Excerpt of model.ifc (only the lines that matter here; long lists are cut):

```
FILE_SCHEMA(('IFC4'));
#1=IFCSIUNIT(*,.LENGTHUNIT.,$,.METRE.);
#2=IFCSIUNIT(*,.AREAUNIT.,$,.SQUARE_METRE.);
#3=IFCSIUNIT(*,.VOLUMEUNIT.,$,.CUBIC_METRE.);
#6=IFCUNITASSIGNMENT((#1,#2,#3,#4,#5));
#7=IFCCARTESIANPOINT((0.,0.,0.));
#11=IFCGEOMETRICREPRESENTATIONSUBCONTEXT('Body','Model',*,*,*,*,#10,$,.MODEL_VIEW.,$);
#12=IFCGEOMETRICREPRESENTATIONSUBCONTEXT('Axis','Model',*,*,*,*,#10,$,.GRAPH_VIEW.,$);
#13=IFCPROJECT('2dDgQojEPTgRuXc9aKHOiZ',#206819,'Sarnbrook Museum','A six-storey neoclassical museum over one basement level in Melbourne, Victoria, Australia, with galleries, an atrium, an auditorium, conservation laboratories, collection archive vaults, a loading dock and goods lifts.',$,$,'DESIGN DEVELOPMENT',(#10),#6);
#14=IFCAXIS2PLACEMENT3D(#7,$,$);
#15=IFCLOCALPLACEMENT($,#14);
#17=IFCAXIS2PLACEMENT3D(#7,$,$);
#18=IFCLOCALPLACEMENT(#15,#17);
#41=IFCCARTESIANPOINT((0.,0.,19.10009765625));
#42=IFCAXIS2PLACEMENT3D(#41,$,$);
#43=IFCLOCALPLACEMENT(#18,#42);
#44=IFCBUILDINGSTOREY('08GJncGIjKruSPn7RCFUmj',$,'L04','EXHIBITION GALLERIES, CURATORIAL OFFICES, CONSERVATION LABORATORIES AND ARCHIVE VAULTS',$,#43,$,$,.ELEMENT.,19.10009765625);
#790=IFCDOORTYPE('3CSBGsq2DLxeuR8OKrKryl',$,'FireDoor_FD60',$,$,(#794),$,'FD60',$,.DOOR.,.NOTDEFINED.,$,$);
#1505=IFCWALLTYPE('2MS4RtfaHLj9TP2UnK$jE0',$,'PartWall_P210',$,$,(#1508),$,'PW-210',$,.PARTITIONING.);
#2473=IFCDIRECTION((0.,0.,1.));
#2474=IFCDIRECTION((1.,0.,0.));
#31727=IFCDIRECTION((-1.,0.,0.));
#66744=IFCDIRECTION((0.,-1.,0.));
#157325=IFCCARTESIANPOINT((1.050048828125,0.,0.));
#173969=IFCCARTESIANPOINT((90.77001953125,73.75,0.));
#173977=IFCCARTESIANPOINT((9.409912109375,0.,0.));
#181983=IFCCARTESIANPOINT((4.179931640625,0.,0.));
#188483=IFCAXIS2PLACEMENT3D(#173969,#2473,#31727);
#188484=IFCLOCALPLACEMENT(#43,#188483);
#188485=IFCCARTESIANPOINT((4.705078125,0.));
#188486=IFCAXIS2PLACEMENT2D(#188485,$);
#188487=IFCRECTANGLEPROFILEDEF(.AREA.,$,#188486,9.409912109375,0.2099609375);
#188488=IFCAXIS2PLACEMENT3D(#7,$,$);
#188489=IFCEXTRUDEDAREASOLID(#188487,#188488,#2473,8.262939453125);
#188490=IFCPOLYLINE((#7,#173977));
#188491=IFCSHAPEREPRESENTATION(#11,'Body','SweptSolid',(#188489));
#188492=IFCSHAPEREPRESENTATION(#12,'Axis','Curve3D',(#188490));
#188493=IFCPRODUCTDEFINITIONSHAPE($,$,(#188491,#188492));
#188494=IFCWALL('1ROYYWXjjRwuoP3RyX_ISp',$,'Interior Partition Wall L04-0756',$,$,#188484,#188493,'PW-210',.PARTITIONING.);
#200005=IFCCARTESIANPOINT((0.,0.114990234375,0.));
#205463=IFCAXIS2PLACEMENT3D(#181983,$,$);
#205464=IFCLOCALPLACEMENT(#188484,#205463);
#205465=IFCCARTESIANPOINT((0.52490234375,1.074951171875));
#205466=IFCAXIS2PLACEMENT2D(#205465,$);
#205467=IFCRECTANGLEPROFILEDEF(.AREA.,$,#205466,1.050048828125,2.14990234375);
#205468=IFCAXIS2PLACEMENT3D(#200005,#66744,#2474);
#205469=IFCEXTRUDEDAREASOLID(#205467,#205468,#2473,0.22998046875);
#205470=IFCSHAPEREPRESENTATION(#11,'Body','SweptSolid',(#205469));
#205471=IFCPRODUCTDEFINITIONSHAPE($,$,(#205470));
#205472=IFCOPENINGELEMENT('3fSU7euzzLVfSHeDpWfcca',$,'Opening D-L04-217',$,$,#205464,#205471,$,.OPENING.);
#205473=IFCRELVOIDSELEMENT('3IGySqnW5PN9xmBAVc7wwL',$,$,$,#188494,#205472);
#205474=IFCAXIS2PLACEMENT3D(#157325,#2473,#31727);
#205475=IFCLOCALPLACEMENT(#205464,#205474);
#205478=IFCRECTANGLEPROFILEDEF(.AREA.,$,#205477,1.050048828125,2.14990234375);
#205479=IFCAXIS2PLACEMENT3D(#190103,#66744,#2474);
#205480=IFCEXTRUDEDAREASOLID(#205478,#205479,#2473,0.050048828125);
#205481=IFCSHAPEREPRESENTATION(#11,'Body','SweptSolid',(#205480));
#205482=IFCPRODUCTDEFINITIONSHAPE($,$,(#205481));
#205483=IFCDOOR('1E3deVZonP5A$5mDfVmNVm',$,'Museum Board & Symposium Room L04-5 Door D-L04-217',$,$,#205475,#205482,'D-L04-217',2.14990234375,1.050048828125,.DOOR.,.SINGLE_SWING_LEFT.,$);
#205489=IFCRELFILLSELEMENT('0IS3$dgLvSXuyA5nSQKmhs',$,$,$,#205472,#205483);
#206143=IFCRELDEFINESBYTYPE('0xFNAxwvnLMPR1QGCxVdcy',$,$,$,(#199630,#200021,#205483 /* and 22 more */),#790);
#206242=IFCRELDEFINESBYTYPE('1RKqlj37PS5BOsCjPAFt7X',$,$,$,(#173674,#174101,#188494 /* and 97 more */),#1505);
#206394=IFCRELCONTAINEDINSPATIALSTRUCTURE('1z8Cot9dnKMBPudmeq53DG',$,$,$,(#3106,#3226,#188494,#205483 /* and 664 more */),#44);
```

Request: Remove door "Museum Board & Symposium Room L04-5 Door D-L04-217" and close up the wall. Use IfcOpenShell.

```python
import ifcopenshell
import ifcopenshell.api.feature
import ifcopenshell.api.root
import ifcopenshell.geom
import ifcopenshell.util.shape

model = ifcopenshell.open("model.ifc")
settings = ifcopenshell.geom.settings()


def volume(element):
    """Net volume in cubic metres, openings subtracted."""
    shape = ifcopenshell.geom.create_shape(settings, element)
    return ifcopenshell.util.shape.get_volume(shape.geometry)


door = model.by_guid("1E3deVZonP5A$5mDfVmNVm")
opening = door.FillsVoids[0].RelatingOpeningElement
wall = opening.VoidsElements[0].RelatingBuildingElement
before = volume(wall)

ifcopenshell.api.root.remove_product(model, product=door)
ifcopenshell.api.feature.remove_feature(model, feature=opening)

after = volume(wall)

print(f"wall volume {before:.3f} -> {after:.3f} m3")

model.write("model_v2.ifc")
```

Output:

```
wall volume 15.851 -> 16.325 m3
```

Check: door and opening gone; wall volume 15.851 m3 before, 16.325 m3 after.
